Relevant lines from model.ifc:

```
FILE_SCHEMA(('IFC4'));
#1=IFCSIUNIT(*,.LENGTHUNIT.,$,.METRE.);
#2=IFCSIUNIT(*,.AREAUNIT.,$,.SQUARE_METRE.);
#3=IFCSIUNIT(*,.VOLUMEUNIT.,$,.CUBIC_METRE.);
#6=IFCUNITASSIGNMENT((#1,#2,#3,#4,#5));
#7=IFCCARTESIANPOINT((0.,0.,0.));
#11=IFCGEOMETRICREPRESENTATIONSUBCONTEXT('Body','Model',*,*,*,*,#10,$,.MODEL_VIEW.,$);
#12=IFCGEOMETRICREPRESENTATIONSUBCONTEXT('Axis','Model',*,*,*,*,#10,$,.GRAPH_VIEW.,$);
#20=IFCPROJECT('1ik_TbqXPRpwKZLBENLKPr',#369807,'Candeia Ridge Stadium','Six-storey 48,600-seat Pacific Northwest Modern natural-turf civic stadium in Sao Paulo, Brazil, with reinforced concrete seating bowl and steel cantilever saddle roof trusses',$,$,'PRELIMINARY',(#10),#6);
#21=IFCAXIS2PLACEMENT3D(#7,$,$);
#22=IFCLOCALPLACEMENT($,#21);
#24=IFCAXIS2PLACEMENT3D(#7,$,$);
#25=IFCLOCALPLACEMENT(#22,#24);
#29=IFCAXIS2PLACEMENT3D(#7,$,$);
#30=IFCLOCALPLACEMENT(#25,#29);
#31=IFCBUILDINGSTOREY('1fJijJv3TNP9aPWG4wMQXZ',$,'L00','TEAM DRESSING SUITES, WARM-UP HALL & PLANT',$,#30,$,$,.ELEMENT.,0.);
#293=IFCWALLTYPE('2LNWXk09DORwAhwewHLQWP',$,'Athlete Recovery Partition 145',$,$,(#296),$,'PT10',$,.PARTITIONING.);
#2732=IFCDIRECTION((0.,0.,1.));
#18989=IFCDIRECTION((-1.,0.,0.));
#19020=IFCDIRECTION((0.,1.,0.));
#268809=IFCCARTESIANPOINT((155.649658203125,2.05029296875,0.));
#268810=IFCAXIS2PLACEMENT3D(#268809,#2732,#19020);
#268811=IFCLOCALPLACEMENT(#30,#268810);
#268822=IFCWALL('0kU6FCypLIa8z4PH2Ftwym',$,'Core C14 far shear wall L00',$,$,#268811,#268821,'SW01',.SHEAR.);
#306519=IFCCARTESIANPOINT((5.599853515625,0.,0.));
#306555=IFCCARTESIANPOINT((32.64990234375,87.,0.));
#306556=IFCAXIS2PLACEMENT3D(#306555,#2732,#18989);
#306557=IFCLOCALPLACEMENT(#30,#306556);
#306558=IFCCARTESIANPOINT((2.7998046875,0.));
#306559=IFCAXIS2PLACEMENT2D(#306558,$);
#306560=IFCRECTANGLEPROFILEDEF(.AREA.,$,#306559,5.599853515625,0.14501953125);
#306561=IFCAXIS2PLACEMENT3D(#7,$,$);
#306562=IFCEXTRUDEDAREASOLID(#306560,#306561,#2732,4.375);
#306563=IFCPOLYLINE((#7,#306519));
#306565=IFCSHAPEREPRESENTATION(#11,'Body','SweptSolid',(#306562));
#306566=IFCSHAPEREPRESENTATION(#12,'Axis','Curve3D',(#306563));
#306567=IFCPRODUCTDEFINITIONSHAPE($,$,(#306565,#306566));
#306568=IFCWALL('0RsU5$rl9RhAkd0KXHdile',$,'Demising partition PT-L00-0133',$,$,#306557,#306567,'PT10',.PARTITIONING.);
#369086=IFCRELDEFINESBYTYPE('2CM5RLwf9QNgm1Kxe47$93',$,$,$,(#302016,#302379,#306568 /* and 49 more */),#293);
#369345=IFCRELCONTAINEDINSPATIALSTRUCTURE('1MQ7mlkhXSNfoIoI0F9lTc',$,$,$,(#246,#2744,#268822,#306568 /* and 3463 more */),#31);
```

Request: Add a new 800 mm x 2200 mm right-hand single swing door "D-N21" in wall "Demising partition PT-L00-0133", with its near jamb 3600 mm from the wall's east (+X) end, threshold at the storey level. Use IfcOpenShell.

```python
import numpy as np
import ifcopenshell
import ifcopenshell.api.feature
import ifcopenshell.api.geometry
import ifcopenshell.api.root
import ifcopenshell.api.spatial
import ifcopenshell.geom
import ifcopenshell.util.element
import ifcopenshell.util.placement
import ifcopenshell.util.representation
import ifcopenshell.util.shape
import ifcopenshell.util.unit

model = ifcopenshell.open("model.ifc")
unit_scale = ifcopenshell.util.unit.calculate_unit_scale(model)
settings = ifcopenshell.geom.settings()


def volume(element):
    """Net volume in cubic metres, openings subtracted."""
    shape = ifcopenshell.geom.create_shape(settings, element)
    return ifcopenshell.util.shape.get_volume(shape.geometry)


wall = model.by_id(306568)
storey = ifcopenshell.util.element.get_container(wall, ifc_class="IfcBuildingStorey")
context = ifcopenshell.util.representation.get_context(model, "Model", "Body", "MODEL_VIEW")
before = volume(wall)

width, height, from_end, sill = 0.8, 2.2, 3.6, 0.0  # metres

# The wall runs along its own X axis, and the end named is its -X end.
wall_shape = ifcopenshell.geom.create_shape(settings, wall)
x, y, z = ifcopenshell.util.shape.get_vertices(wall_shape.geometry).T
start = x.min() + from_end
face, thickness = float(y.min()), float(y.max() - y.min())
wall_matrix = ifcopenshell.util.placement.get_local_placement(wall.ObjectPlacement)
level = ifcopenshell.util.placement.get_local_placement(storey.ObjectPlacement)[2, 3]


def in_wall(x, y):
    """Placement at x, y metres in the wall's axes, at sill height."""
    matrix = wall_matrix.copy()
    matrix[:, 3] = wall_matrix @ np.array([x / unit_scale, y / unit_scale, 0.0, 1.0])
    matrix[2, 3] = level + sill / unit_scale
    return matrix


# Opening: a box that overshoots both wall faces by 50 mm.
opening = ifcopenshell.api.root.create_entity(model, ifc_class="IfcOpeningElement", predefined_type="OPENING")
box = ifcopenshell.api.geometry.add_wall_representation(
    model, context=context, length=width, height=height, thickness=thickness + 0.1
)
ifcopenshell.api.geometry.assign_representation(model, product=opening, representation=box)
ifcopenshell.api.geometry.edit_object_placement(model, product=opening, matrix=in_wall(start, face - 0.05), is_si=False)
ifcopenshell.api.feature.add_feature(model, feature=opening, element=wall)

door = ifcopenshell.api.root.create_entity(model, ifc_class="IfcDoor", name="D-N21", predefined_type="DOOR")
door.OverallWidth, door.OverallHeight = width / unit_scale, height / unit_scale
door.OperationType = "SINGLE_SWING_RIGHT"
body = ifcopenshell.api.geometry.add_door_representation(
    model,
    context=context,
    overall_width=door.OverallWidth,
    overall_height=door.OverallHeight,
    operation_type="SINGLE_SWING_RIGHT",
    lining_properties={"LiningDepth": thickness / unit_scale, "ThresholdDepth": thickness / unit_scale},
)
ifcopenshell.api.geometry.assign_representation(model, product=door, representation=body)
ifcopenshell.api.spatial.assign_container(model, products=[door], relating_structure=storey)
ifcopenshell.api.feature.add_filling(model, opening=opening, element=door)

# The lining spans the wall, so the door starts at the wall face.
ifcopenshell.api.geometry.edit_object_placement(model, product=door, matrix=in_wall(start, face), is_si=False)

after = volume(wall)

print(f"wall volume {before:.3f} -> {after:.3f} m3")

model.write("model_updated.ifc")
```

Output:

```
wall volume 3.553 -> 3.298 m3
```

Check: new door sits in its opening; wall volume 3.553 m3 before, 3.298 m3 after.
